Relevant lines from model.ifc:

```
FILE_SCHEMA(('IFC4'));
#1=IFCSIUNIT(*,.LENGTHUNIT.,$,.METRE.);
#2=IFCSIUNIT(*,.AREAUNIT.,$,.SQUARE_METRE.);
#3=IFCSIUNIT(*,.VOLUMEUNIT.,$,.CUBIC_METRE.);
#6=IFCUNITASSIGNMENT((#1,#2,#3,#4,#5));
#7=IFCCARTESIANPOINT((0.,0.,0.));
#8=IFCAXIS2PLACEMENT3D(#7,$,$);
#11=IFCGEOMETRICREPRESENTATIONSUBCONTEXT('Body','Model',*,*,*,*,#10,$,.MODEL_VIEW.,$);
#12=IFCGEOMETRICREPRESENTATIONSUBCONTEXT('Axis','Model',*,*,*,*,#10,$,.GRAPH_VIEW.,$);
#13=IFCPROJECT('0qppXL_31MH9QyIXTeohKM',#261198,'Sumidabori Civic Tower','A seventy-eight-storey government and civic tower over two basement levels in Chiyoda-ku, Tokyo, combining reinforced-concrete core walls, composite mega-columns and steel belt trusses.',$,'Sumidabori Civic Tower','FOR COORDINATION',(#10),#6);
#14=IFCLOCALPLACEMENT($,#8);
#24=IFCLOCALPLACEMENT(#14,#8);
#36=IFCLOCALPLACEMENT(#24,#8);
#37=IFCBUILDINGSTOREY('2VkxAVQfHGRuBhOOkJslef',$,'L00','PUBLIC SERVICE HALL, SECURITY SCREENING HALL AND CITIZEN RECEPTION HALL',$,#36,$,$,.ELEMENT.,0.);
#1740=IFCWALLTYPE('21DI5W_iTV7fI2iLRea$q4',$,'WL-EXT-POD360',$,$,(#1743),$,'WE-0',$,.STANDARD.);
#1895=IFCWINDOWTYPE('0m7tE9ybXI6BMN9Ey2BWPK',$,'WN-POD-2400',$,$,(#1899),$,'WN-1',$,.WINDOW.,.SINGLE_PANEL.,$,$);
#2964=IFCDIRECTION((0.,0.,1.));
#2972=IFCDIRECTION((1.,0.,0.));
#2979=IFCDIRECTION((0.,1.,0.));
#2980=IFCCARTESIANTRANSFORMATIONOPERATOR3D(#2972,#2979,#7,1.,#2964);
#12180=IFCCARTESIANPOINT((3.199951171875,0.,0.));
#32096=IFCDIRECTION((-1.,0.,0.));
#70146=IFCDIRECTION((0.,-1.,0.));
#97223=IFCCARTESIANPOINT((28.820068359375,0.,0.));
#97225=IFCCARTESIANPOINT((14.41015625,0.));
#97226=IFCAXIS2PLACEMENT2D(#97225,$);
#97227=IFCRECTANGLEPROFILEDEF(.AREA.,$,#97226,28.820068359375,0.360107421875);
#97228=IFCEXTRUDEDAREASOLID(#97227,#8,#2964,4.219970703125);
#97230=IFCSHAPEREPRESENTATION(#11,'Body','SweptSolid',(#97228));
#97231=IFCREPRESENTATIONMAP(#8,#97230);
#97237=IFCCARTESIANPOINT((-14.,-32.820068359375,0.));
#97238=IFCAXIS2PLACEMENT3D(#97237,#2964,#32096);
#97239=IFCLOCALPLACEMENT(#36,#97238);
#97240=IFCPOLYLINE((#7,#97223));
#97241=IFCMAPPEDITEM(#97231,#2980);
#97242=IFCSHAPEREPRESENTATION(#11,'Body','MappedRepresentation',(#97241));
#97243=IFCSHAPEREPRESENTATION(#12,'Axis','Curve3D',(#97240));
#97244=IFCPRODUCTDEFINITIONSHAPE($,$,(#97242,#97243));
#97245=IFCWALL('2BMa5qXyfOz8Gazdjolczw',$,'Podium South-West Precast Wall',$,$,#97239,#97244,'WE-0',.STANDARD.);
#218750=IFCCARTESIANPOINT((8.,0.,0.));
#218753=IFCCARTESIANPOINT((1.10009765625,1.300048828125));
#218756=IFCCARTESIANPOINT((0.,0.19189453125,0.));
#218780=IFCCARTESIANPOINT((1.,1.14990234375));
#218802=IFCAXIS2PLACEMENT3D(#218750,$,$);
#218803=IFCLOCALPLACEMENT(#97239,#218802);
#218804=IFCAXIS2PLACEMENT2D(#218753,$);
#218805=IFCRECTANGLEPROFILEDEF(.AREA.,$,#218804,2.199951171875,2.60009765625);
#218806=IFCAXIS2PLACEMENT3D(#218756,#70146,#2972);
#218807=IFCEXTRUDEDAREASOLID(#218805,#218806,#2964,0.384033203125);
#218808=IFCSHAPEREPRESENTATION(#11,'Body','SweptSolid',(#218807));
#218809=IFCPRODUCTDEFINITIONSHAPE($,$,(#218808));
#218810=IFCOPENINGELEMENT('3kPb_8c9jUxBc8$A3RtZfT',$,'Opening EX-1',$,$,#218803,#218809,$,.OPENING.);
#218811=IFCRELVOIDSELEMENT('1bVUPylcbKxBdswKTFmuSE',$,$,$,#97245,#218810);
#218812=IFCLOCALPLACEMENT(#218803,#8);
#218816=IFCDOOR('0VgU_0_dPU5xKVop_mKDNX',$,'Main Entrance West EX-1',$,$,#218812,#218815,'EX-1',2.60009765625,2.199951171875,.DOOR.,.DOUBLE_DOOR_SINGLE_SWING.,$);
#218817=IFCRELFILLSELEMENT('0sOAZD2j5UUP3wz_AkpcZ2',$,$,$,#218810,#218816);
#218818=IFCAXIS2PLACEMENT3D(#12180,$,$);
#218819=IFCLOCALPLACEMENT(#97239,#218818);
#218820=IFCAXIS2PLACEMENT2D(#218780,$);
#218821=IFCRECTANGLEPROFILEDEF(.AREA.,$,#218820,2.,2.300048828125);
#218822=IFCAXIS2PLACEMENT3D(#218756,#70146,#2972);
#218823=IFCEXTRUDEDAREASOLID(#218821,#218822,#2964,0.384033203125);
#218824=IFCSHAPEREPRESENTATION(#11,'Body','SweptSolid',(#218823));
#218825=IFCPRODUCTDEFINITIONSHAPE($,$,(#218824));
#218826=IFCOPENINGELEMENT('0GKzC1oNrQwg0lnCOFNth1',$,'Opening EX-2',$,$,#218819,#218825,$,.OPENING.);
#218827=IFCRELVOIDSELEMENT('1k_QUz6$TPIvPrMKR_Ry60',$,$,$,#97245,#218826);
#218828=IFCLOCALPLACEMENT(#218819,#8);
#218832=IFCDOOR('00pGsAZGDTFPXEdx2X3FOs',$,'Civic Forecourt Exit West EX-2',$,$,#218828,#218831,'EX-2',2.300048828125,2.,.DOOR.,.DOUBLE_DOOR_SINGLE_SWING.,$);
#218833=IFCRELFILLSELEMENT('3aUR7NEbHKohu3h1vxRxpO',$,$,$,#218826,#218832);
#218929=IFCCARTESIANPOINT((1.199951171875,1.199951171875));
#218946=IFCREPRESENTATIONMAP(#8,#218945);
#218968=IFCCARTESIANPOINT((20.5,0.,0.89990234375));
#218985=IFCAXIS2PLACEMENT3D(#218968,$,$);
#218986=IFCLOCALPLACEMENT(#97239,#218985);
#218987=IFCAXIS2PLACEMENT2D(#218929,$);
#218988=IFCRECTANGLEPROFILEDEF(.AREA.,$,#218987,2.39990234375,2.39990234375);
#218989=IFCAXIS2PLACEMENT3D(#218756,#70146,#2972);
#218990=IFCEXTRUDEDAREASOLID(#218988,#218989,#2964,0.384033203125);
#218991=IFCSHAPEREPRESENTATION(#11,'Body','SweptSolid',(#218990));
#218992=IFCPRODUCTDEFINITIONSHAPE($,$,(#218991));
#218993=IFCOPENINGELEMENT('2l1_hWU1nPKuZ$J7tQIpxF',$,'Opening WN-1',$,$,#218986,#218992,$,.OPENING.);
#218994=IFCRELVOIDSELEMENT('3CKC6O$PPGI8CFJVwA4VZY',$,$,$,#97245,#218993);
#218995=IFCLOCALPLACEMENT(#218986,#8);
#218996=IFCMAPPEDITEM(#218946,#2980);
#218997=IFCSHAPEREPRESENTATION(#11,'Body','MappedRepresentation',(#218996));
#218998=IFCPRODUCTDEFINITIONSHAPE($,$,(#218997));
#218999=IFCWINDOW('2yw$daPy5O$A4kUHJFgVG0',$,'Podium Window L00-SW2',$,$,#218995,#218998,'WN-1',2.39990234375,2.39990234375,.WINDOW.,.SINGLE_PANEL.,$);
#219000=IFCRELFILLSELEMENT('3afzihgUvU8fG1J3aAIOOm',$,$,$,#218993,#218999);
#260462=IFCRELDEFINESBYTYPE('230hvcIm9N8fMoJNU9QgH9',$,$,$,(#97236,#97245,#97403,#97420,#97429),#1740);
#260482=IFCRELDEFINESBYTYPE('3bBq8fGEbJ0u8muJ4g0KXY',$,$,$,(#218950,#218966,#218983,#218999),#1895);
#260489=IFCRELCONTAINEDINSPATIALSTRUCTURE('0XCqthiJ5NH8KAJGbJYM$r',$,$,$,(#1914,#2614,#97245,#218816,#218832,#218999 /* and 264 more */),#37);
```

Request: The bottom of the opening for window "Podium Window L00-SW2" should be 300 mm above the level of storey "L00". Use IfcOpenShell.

```python
import numpy as np
import ifcopenshell
import ifcopenshell.api.geometry
import ifcopenshell.geom
import ifcopenshell.util.element
import ifcopenshell.util.placement
import ifcopenshell.util.shape
import ifcopenshell.util.unit

model = ifcopenshell.open("model.ifc")
unit_scale = ifcopenshell.util.unit.calculate_unit_scale(model)

window = model.by_guid("2yw$daPy5O$A4kUHJFgVG0")
opening = window.FillsVoids[0].RelatingOpeningElement
storey = ifcopenshell.util.element.get_container(window, ifc_class="IfcBuildingStorey")
level = ifcopenshell.util.placement.get_local_placement(storey.ObjectPlacement)[2, 3]

# The opening's origin need not be at the sill, so measure its lowest point.
shape = ifcopenshell.geom.create_shape(ifcopenshell.geom.settings(), opening)
bottom = ifcopenshell.util.shape.get_shape_bottom_elevation(shape, shape.geometry) / unit_scale
dz = level + 0.3 / unit_scale - bottom

shift = np.array([0.0, 0.0, dz])
# The window is placed relative to its opening, so it follows when the opening moves.
matrix = ifcopenshell.util.placement.get_local_placement(opening.ObjectPlacement)
matrix[:3, 3] += shift
ifcopenshell.api.geometry.edit_object_placement(
    model, product=opening, matrix=matrix, is_si=False, should_transform_children=True
)

print(f"moved by {dz * unit_scale:+.3f} m")

model.write("model_edited.ifc")
```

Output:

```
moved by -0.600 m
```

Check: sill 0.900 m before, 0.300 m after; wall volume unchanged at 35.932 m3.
